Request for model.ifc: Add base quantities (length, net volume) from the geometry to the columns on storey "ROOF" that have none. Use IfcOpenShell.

First a look at what the model holds.

```python
import ifcopenshell
import ifcopenshell.util.element
import ifcopenshell.util.unit

model = ifcopenshell.open("model.ifc")
print(model.schema)
for unit_type in ("LENGTHUNIT", "AREAUNIT", "VOLUMEUNIT"):
    print(unit_type, ifcopenshell.util.unit.calculate_unit_scale(model, unit_type))
storey = next(s for s in model.by_type("IfcBuildingStorey") if s.Name == "ROOF")
columns = [e for e in ifcopenshell.util.element.get_decomposition(storey) if e.is_a("IfcColumn")]
for e in sorted(columns, key=lambda e: e.id()):
    print(e.id(), e.is_a(), e.Name, list(ifcopenshell.util.element.get_psets(e, qtos_only=True)), sep=" | ")
```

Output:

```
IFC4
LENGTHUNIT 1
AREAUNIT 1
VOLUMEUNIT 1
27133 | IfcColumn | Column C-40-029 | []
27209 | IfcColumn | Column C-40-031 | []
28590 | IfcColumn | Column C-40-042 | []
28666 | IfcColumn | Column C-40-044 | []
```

```python
import ifcopenshell
import ifcopenshell.api.pset
import ifcopenshell.geom
import ifcopenshell.util.element
import ifcopenshell.util.shape
import ifcopenshell.util.unit

model = ifcopenshell.open("model.ifc")
unit_scale = ifcopenshell.util.unit.calculate_unit_scale(model)
volume_scale = ifcopenshell.util.unit.calculate_unit_scale(model, "VOLUMEUNIT")
settings = ifcopenshell.geom.settings()

storey = next(s for s in model.by_type("IfcBuildingStorey") if s.Name == "ROOF")
columns = [e for e in ifcopenshell.util.element.get_decomposition(storey) if e.is_a("IfcColumn")]

for e in sorted(columns, key=lambda e: e.id()):
    if ifcopenshell.util.element.get_psets(e, qtos_only=True, should_inherit=False):
        continue
    # Geometry comes back in metres, in the element's own axes.
    shape = ifcopenshell.geom.create_shape(settings, e)
    values = {
        "Length": ifcopenshell.util.shape.get_z(shape.geometry) / unit_scale,
        "NetVolume": ifcopenshell.util.shape.get_volume(shape.geometry) / volume_scale,
    }
    qto = ifcopenshell.api.pset.add_qto(model, product=e, name="Qto_ColumnBaseQuantities")
    ifcopenshell.api.pset.edit_qto(model, qto=qto, properties=values)
    print(e.id(), {k: round(v, 3) for k, v in values.items()})

model.write("model_v2.ifc")
```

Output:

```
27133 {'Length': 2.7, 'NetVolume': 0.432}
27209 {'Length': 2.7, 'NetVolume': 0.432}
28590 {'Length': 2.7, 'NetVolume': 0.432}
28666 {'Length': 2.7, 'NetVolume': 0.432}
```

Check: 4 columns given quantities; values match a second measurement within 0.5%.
